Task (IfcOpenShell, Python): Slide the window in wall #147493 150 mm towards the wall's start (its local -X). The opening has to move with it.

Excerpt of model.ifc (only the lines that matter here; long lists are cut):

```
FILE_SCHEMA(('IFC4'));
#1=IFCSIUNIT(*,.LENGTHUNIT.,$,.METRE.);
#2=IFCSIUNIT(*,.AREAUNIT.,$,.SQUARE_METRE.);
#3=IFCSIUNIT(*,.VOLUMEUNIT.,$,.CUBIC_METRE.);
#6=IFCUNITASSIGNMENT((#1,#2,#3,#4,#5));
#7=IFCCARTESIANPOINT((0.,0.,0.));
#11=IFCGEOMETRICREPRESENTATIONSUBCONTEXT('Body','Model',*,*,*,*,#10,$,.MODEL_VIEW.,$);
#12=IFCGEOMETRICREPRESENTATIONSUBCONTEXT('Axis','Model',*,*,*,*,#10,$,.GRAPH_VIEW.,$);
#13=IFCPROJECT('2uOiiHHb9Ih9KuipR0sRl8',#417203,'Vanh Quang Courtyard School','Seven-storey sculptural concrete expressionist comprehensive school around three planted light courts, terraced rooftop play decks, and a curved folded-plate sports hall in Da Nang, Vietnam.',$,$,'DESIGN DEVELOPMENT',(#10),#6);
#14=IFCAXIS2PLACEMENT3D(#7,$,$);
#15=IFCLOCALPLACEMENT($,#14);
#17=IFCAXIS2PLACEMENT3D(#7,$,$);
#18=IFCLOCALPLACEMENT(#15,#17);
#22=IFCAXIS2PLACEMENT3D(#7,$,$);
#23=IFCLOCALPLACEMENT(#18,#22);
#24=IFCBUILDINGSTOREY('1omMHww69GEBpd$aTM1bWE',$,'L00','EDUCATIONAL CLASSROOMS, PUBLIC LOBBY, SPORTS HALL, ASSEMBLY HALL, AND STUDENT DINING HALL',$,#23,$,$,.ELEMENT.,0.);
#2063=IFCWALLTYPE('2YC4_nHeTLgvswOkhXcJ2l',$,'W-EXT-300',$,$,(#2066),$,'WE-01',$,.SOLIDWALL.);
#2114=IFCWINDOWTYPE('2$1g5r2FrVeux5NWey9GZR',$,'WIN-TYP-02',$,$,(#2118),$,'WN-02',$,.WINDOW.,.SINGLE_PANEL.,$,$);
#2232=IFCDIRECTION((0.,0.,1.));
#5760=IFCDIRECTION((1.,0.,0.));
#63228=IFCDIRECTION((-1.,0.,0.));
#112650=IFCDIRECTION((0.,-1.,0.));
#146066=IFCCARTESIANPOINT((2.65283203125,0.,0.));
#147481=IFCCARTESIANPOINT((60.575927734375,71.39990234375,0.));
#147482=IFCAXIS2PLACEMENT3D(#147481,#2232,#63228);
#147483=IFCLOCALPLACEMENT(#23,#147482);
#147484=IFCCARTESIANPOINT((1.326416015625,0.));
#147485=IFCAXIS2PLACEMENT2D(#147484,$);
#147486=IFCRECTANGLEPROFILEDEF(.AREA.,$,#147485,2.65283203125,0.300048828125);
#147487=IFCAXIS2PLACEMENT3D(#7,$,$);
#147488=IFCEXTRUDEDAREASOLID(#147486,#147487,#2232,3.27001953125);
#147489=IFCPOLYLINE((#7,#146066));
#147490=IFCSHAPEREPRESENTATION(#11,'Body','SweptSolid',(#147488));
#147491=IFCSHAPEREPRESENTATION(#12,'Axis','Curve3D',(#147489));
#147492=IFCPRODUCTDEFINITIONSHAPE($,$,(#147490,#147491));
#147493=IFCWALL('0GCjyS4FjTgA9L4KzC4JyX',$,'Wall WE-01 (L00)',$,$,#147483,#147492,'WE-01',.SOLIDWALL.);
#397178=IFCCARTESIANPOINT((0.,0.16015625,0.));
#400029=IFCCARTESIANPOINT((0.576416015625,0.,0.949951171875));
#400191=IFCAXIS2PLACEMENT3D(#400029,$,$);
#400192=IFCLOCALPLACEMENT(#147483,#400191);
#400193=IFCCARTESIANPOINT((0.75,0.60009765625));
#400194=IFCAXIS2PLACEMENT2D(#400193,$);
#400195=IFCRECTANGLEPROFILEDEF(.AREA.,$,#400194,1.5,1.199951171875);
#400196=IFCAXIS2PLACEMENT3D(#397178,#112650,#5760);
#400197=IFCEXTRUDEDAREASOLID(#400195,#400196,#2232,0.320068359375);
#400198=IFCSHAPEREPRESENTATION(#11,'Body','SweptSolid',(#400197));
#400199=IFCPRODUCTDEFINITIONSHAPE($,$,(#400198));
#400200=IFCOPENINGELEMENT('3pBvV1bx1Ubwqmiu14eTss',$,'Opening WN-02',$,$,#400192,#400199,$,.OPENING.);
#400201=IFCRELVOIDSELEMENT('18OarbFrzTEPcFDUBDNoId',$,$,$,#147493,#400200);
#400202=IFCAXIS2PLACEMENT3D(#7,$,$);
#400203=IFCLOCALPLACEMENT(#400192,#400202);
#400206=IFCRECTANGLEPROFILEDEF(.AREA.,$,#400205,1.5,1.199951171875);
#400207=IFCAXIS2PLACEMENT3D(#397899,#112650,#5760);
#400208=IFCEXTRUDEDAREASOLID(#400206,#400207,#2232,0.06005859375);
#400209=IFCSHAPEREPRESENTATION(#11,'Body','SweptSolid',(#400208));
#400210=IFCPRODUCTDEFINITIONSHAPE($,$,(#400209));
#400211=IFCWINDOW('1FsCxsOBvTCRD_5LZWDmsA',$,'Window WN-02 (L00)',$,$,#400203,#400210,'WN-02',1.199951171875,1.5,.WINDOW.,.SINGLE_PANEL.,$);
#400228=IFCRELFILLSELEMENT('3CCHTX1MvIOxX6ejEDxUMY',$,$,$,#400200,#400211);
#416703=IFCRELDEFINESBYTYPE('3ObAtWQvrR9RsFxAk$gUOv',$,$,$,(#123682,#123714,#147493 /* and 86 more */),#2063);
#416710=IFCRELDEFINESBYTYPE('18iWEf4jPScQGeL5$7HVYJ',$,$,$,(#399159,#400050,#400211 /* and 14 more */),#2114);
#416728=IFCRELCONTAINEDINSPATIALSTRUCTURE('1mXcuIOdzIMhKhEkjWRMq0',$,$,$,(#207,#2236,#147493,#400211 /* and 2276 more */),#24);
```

```python
import ifcopenshell
import ifcopenshell.api.geometry
import ifcopenshell.util.placement
import ifcopenshell.util.unit

model = ifcopenshell.open("model.ifc")
unit_scale = ifcopenshell.util.unit.calculate_unit_scale(model)

window = model.by_guid("1FsCxsOBvTCRD_5LZWDmsA")
opening = window.FillsVoids[0].RelatingOpeningElement
wall = opening.VoidsElements[0].RelatingBuildingElement

wall_matrix = ifcopenshell.util.placement.get_local_placement(wall.ObjectPlacement)
shift = wall_matrix[:3, 0] * -0.15 / unit_scale
before = ifcopenshell.util.placement.get_local_placement(window.ObjectPlacement)[:3, 3].copy()

# The window is placed relative to its opening, so it follows when the opening moves.
matrix = ifcopenshell.util.placement.get_local_placement(opening.ObjectPlacement)
matrix[:3, 3] += shift
ifcopenshell.api.geometry.edit_object_placement(
    model, product=opening, matrix=matrix, is_si=False, should_transform_children=True
)

after = ifcopenshell.util.placement.get_local_placement(window.ObjectPlacement)[:3, 3]
print("window moved by", (after - before).round(3) + 0.0)

model.write("model-out.ifc")
```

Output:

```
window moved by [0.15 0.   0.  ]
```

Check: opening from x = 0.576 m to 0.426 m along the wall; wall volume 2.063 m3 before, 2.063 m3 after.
